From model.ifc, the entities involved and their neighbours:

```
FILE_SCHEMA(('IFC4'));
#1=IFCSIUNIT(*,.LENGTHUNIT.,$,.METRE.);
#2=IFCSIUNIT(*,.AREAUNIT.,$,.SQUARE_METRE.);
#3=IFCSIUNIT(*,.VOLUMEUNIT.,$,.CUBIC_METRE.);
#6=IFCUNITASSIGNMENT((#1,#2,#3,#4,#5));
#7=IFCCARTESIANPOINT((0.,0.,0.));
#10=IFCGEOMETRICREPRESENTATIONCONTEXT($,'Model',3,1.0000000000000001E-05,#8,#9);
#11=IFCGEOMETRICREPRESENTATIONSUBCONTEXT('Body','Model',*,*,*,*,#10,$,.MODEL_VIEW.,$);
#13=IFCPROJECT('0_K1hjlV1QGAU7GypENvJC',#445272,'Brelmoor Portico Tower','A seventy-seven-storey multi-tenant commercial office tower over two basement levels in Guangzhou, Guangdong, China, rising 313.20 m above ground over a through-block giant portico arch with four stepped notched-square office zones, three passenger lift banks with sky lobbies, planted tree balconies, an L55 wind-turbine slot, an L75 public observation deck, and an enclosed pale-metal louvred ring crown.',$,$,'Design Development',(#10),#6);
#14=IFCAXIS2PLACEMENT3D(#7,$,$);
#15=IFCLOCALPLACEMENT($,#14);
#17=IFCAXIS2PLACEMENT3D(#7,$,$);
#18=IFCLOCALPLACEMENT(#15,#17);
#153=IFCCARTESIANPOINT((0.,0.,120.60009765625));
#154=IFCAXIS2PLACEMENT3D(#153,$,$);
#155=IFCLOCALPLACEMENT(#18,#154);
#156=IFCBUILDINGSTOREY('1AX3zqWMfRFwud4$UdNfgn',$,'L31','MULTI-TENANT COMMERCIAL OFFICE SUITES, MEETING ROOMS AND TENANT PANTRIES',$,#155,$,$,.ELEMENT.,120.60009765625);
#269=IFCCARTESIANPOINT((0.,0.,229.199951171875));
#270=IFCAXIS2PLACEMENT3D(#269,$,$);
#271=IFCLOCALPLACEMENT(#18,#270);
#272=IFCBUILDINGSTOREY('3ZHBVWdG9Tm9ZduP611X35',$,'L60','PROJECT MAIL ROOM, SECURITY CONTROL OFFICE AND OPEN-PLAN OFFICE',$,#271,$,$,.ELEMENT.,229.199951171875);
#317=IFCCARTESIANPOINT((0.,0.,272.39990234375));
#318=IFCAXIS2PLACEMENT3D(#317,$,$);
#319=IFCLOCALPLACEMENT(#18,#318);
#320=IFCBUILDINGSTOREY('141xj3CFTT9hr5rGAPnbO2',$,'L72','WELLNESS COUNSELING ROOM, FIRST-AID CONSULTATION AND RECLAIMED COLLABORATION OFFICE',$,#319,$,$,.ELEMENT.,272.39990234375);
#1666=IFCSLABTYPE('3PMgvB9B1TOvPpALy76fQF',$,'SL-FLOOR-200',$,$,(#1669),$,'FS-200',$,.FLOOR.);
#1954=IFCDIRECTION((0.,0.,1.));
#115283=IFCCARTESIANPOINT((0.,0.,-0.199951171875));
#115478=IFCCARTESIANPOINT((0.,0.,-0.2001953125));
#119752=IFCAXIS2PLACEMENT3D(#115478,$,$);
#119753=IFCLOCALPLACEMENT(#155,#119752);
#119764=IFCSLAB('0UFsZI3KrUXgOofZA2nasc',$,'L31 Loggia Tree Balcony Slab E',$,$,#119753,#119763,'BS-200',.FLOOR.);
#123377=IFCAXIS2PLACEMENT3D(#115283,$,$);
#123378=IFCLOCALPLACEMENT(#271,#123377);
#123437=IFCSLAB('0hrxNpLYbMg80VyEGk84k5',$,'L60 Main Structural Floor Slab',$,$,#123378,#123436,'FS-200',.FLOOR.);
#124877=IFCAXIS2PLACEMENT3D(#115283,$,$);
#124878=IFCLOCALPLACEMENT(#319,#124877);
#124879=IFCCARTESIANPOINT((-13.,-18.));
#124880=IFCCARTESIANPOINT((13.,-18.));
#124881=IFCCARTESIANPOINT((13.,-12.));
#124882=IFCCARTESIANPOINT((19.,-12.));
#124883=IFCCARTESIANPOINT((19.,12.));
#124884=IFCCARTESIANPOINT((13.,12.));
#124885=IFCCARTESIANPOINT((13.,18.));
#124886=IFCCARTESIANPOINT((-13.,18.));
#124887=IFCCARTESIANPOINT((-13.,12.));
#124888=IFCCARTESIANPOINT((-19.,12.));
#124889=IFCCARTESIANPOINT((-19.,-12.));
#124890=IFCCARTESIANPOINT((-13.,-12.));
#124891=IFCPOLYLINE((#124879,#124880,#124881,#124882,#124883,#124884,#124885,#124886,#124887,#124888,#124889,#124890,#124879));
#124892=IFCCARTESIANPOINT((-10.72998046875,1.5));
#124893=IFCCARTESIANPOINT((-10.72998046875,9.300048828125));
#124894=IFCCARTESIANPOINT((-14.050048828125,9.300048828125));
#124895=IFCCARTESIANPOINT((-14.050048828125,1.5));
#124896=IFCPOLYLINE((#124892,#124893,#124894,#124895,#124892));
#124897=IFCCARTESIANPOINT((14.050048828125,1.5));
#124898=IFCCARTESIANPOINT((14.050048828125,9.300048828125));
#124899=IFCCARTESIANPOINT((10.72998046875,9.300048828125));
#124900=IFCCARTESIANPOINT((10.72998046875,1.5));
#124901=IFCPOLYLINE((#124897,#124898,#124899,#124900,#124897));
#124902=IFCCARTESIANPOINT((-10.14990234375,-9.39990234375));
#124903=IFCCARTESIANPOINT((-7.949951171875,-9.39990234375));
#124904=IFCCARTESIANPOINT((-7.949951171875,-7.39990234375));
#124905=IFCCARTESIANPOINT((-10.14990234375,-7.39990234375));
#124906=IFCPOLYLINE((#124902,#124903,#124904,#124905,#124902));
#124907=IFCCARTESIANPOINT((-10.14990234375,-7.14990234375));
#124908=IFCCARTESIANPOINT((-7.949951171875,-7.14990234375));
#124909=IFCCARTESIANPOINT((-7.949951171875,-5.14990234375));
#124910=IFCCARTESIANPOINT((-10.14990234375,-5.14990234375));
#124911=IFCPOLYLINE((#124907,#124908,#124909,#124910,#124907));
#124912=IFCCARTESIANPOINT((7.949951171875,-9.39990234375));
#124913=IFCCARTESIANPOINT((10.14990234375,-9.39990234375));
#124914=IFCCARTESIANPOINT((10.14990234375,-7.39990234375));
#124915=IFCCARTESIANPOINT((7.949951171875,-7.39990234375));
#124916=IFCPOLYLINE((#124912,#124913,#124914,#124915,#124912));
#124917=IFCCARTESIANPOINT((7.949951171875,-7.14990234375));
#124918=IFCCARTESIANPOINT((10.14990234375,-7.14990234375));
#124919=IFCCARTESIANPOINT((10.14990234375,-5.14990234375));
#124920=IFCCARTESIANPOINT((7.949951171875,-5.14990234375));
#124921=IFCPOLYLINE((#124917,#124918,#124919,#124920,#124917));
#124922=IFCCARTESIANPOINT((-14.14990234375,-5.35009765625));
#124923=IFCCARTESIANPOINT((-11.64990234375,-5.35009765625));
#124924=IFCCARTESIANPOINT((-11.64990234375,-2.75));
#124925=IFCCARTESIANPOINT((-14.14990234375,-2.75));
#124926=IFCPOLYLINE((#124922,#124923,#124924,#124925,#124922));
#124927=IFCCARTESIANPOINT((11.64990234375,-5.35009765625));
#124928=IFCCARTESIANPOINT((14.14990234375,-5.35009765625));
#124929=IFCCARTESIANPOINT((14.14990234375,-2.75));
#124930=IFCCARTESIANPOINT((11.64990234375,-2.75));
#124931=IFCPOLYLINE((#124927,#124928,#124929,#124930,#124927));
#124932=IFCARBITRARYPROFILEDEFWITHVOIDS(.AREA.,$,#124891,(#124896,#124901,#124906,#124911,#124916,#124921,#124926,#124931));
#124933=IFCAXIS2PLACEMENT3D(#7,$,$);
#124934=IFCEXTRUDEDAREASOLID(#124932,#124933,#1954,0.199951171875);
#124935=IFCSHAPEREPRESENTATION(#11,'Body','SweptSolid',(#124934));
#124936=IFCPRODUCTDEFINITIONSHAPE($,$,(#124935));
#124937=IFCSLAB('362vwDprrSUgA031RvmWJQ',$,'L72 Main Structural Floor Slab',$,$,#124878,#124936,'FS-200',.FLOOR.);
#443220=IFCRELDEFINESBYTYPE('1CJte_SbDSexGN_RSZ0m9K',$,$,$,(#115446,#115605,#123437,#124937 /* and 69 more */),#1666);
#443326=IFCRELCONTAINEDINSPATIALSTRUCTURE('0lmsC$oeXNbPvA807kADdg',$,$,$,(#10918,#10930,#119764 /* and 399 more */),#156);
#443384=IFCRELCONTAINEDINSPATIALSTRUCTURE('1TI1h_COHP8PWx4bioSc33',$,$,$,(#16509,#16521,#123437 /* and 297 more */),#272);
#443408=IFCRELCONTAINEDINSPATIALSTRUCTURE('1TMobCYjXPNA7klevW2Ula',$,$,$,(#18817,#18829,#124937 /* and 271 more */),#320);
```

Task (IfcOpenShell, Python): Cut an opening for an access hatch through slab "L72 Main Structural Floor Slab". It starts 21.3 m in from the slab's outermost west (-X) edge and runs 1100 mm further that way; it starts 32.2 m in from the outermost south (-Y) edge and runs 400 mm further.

```python
import numpy as np
import ifcopenshell
import ifcopenshell.api.feature
import ifcopenshell.api.geometry
import ifcopenshell.api.root
import ifcopenshell.geom
import ifcopenshell.util.placement
import ifcopenshell.util.representation
import ifcopenshell.util.shape
import ifcopenshell.util.unit

model = ifcopenshell.open("model.ifc")
unit_scale = ifcopenshell.util.unit.calculate_unit_scale(model)
settings = ifcopenshell.geom.settings()


def volume(element):
    """Net volume in cubic metres, openings subtracted."""
    shape = ifcopenshell.geom.create_shape(settings, element)
    return ifcopenshell.util.shape.get_volume(shape.geometry)


slab = model.by_guid("362vwDprrSUgA031RvmWJQ")
before = volume(slab)

# Extent in the slab's own axes, in metres. The edges named are its -X and -Y sides.
slab_shape = ifcopenshell.geom.create_shape(settings, slab)
vertices = ifcopenshell.util.shape.get_vertices(slab_shape.geometry)
x_min, y_min, bottom = vertices.min(axis=0)
top = vertices[:, 2].max()

opening = ifcopenshell.api.root.create_entity(model, ifc_class="IfcOpeningElement", name="Access hatch opening", predefined_type="OPENING")
context = ifcopenshell.util.representation.get_context(model, "Model", "Body", "MODEL_VIEW")
width, depth = 1.1, 0.4
outline = [(0.0, 0.0), (width, 0.0), (width, depth), (0.0, depth), (0.0, 0.0)]
# Overshoot both faces by 50 mm so the cut is clean.
shape = ifcopenshell.api.geometry.add_slab_representation(
    model, context=context, depth=top - bottom + 0.1, polyline=outline
)
ifcopenshell.api.geometry.assign_representation(model, product=opening, representation=shape)

matrix = ifcopenshell.util.placement.get_local_placement(slab.ObjectPlacement)
matrix[:, 3] = matrix @ np.append(np.array([x_min + 21.3, y_min + 32.2, bottom - 0.05]) / unit_scale, 1.0)
ifcopenshell.api.geometry.edit_object_placement(model, product=opening, matrix=matrix, is_si=False)
ifcopenshell.api.feature.add_feature(model, feature=opening, element=slab)

after = volume(slab)

print(f"slab volume {before:.3f} -> {after:.3f} m3")

model.write("model-out.ifc")
```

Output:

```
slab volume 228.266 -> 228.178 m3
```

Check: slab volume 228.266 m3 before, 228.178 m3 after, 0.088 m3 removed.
